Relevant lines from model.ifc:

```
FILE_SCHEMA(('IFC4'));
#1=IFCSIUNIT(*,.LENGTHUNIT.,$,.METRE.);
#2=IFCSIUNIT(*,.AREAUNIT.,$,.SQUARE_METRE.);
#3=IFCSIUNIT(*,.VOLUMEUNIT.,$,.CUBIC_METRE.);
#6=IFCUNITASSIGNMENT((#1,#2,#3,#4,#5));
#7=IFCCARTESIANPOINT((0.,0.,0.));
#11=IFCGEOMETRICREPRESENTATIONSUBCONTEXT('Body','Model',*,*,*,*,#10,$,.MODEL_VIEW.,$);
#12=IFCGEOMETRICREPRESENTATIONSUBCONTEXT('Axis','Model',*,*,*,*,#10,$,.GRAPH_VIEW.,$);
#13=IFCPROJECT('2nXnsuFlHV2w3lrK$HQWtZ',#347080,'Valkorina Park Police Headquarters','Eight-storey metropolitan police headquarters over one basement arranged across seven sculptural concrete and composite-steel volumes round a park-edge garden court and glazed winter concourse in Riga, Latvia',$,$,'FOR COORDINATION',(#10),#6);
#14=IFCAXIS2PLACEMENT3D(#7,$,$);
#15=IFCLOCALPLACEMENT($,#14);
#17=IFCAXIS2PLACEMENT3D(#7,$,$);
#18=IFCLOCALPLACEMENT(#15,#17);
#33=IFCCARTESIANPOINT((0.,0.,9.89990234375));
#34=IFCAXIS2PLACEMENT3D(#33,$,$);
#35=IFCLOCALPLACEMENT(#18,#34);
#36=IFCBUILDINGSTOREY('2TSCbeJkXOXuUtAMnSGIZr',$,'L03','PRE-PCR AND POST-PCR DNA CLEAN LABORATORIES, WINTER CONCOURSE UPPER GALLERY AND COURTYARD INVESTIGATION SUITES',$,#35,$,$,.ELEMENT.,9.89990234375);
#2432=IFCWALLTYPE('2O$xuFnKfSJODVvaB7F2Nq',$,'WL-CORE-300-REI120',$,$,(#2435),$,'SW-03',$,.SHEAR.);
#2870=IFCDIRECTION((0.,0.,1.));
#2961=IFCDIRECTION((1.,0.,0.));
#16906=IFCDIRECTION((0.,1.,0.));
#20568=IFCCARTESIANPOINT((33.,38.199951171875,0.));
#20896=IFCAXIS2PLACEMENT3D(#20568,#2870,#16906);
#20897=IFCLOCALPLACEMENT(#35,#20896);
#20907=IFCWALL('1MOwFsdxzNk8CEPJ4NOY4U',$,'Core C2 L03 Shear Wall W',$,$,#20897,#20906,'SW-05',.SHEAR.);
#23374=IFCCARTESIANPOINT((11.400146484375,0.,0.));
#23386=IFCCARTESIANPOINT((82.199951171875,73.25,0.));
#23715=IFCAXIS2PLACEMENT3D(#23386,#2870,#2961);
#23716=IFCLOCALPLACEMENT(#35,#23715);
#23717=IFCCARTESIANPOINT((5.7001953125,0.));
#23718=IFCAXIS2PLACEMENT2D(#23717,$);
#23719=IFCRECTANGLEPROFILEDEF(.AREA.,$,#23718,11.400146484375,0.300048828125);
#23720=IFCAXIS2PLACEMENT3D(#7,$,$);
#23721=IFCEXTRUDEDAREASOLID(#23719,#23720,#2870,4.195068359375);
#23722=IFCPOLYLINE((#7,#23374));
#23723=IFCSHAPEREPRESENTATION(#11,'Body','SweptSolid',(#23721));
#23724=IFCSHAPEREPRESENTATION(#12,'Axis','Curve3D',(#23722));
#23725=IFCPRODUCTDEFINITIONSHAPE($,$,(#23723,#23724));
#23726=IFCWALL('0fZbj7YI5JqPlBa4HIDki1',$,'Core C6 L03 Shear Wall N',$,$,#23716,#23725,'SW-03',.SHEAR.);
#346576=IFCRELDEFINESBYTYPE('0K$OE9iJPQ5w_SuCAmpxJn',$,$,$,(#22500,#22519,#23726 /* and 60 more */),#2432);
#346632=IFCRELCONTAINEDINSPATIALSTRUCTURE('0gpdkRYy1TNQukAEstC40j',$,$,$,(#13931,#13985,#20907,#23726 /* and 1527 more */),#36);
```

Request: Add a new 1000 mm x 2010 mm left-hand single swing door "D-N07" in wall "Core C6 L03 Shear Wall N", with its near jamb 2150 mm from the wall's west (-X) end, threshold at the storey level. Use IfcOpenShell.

```python
import numpy as np
import ifcopenshell
import ifcopenshell.api.feature
import ifcopenshell.api.geometry
import ifcopenshell.api.root
import ifcopenshell.api.spatial
import ifcopenshell.geom
import ifcopenshell.util.element
import ifcopenshell.util.placement
import ifcopenshell.util.representation
import ifcopenshell.util.shape
import ifcopenshell.util.unit

model = ifcopenshell.open("model.ifc")
unit_scale = ifcopenshell.util.unit.calculate_unit_scale(model)
settings = ifcopenshell.geom.settings()


def volume(element):
    """Net volume in cubic metres, openings subtracted."""
    shape = ifcopenshell.geom.create_shape(settings, element)
    return ifcopenshell.util.shape.get_volume(shape.geometry)


wall = model.by_guid("0fZbj7YI5JqPlBa4HIDki1")
storey = ifcopenshell.util.element.get_container(wall, ifc_class="IfcBuildingStorey")
context = ifcopenshell.util.representation.get_context(model, "Model", "Body", "MODEL_VIEW")
before = volume(wall)

width, height, from_end, sill = 1, 2.01, 2.15, 0.0  # metres

# The wall runs along its own X axis, and the end named is its -X end.
wall_shape = ifcopenshell.geom.create_shape(settings, wall)
x, y, z = ifcopenshell.util.shape.get_vertices(wall_shape.geometry).T
start = x.min() + from_end
face, thickness = float(y.min()), float(y.max() - y.min())
wall_matrix = ifcopenshell.util.placement.get_local_placement(wall.ObjectPlacement)
level = ifcopenshell.util.placement.get_local_placement(storey.ObjectPlacement)[2, 3]


def in_wall(x, y):
    """Placement at x, y metres in the wall's axes, at sill height."""
    matrix = wall_matrix.copy()
    matrix[:, 3] = wall_matrix @ np.array([x / unit_scale, y / unit_scale, 0.0, 1.0])
    matrix[2, 3] = level + sill / unit_scale
    return matrix


# Opening: a box that overshoots both wall faces by 50 mm.
opening = ifcopenshell.api.root.create_entity(model, ifc_class="IfcOpeningElement", predefined_type="OPENING")
box = ifcopenshell.api.geometry.add_wall_representation(
    model, context=context, length=width, height=height, thickness=thickness + 0.1
)
ifcopenshell.api.geometry.assign_representation(model, product=opening, representation=box)
ifcopenshell.api.geometry.edit_object_placement(model, product=opening, matrix=in_wall(start, face - 0.05), is_si=False)
ifcopenshell.api.feature.add_feature(model, feature=opening, element=wall)

door = ifcopenshell.api.root.create_entity(model, ifc_class="IfcDoor", name="D-N07", predefined_type="DOOR")
door.OverallWidth, door.OverallHeight = width / unit_scale, height / unit_scale
door.OperationType = "SINGLE_SWING_LEFT"
body = ifcopenshell.api.geometry.add_door_representation(
    model,
    context=context,
    overall_width=door.OverallWidth,
    overall_height=door.OverallHeight,
    operation_type="SINGLE_SWING_LEFT",
    lining_properties={"LiningDepth": thickness / unit_scale, "ThresholdDepth": thickness / unit_scale},
)
ifcopenshell.api.geometry.assign_representation(model, product=door, representation=body)
ifcopenshell.api.spatial.assign_container(model, products=[door], relating_structure=storey)
ifcopenshell.api.feature.add_filling(model, opening=opening, element=door)

# The lining spans the wall, so the door starts at the wall face.
ifcopenshell.api.geometry.edit_object_placement(model, product=door, matrix=in_wall(start, face), is_si=False)

after = volume(wall)

print(f"wall volume {before:.3f} -> {after:.3f} m3")

model.write("model_v2.ifc")
```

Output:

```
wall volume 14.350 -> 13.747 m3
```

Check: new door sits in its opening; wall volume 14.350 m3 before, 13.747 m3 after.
